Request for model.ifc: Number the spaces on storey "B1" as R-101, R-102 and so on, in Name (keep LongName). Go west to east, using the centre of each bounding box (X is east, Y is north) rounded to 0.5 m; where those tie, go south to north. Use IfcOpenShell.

First a look at what the model holds.

```python
import ifcopenshell
import ifcopenshell.util.element
import ifcopenshell.util.placement

model = ifcopenshell.open("model.ifc")
print(model.schema)
storey = next(s for s in model.by_type("IfcBuildingStorey") if s.Name == "B1")
spaces = [e for e in ifcopenshell.util.element.get_decomposition(storey) if e.is_a("IfcSpace")]
for e in sorted(spaces, key=lambda e: e.id()):
    origin = ifcopenshell.util.placement.get_local_placement(e.ObjectPlacement)[:3, 3]
    print(e.id(), e.Name, e.LongName, origin.round(2) + 0.0, sep=" | ")
```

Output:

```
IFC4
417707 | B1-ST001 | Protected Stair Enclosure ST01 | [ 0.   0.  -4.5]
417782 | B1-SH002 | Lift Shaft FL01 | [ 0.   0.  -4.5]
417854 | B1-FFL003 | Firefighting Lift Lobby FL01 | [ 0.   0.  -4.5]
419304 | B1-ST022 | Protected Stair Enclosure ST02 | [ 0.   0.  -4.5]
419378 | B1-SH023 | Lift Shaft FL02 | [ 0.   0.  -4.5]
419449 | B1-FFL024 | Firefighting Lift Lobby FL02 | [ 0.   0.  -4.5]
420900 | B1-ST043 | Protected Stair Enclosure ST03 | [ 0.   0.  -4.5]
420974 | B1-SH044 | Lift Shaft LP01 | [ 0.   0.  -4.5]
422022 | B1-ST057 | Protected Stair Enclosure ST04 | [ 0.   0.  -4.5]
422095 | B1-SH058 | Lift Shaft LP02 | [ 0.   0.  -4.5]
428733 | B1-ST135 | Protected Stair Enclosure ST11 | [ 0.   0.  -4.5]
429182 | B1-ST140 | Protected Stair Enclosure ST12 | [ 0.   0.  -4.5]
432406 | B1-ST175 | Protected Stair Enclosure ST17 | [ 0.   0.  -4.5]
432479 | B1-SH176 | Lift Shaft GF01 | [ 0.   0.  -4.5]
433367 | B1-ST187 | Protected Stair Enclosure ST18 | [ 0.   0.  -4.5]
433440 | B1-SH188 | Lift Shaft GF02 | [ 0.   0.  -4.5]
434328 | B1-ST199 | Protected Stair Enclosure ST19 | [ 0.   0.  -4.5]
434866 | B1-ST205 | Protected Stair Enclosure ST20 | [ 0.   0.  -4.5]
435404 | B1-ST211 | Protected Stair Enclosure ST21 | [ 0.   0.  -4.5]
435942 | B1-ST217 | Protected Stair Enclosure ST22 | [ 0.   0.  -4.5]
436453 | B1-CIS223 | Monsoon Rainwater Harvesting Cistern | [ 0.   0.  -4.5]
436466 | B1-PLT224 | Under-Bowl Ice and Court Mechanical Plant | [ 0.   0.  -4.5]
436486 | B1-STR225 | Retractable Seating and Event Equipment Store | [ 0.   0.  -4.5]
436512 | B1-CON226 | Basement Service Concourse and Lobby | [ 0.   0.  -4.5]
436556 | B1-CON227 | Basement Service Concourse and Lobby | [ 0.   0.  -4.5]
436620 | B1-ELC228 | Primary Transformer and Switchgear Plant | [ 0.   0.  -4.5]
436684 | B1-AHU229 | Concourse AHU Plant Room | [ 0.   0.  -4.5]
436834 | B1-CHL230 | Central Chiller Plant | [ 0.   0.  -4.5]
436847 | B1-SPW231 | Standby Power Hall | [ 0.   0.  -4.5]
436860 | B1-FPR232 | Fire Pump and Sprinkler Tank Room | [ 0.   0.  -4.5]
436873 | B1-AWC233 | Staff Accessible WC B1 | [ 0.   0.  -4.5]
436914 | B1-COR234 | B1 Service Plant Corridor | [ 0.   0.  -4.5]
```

```python
import ifcopenshell
import ifcopenshell.geom
import ifcopenshell.util.element
import ifcopenshell.util.shape

model = ifcopenshell.open("model.ifc")
settings = ifcopenshell.geom.settings()
settings.set("use-world-coords", True)


def centre(element):
    shape = ifcopenshell.geom.create_shape(settings, element)
    return ifcopenshell.util.shape.get_bbox_centroid(shape.geometry)


storey = next(s for s in model.by_type("IfcBuildingStorey") if s.Name == "B1")
spaces = [e for e in ifcopenshell.util.element.get_decomposition(storey) if e.is_a("IfcSpace")]

# Insertion points can sit at a corner or the storey origin, so sort by the geometry (in metres).
centres = {e: centre(e) for e in spaces}
spaces.sort(key=lambda e: (round(centres[e][0] / 0.5), centres[e][1]))

for i, e in enumerate(spaces, start=1):
    number = f"R-1{i:02d}"
    e.Name = number
    print(e.id(), number)

model.write("model-out.ifc")
```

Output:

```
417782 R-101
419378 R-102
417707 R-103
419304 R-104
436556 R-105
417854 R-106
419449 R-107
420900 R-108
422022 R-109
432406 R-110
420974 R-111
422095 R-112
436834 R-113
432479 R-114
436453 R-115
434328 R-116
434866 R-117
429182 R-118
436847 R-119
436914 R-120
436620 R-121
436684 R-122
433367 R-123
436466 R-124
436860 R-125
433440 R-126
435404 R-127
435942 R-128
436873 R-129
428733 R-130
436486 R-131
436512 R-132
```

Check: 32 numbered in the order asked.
